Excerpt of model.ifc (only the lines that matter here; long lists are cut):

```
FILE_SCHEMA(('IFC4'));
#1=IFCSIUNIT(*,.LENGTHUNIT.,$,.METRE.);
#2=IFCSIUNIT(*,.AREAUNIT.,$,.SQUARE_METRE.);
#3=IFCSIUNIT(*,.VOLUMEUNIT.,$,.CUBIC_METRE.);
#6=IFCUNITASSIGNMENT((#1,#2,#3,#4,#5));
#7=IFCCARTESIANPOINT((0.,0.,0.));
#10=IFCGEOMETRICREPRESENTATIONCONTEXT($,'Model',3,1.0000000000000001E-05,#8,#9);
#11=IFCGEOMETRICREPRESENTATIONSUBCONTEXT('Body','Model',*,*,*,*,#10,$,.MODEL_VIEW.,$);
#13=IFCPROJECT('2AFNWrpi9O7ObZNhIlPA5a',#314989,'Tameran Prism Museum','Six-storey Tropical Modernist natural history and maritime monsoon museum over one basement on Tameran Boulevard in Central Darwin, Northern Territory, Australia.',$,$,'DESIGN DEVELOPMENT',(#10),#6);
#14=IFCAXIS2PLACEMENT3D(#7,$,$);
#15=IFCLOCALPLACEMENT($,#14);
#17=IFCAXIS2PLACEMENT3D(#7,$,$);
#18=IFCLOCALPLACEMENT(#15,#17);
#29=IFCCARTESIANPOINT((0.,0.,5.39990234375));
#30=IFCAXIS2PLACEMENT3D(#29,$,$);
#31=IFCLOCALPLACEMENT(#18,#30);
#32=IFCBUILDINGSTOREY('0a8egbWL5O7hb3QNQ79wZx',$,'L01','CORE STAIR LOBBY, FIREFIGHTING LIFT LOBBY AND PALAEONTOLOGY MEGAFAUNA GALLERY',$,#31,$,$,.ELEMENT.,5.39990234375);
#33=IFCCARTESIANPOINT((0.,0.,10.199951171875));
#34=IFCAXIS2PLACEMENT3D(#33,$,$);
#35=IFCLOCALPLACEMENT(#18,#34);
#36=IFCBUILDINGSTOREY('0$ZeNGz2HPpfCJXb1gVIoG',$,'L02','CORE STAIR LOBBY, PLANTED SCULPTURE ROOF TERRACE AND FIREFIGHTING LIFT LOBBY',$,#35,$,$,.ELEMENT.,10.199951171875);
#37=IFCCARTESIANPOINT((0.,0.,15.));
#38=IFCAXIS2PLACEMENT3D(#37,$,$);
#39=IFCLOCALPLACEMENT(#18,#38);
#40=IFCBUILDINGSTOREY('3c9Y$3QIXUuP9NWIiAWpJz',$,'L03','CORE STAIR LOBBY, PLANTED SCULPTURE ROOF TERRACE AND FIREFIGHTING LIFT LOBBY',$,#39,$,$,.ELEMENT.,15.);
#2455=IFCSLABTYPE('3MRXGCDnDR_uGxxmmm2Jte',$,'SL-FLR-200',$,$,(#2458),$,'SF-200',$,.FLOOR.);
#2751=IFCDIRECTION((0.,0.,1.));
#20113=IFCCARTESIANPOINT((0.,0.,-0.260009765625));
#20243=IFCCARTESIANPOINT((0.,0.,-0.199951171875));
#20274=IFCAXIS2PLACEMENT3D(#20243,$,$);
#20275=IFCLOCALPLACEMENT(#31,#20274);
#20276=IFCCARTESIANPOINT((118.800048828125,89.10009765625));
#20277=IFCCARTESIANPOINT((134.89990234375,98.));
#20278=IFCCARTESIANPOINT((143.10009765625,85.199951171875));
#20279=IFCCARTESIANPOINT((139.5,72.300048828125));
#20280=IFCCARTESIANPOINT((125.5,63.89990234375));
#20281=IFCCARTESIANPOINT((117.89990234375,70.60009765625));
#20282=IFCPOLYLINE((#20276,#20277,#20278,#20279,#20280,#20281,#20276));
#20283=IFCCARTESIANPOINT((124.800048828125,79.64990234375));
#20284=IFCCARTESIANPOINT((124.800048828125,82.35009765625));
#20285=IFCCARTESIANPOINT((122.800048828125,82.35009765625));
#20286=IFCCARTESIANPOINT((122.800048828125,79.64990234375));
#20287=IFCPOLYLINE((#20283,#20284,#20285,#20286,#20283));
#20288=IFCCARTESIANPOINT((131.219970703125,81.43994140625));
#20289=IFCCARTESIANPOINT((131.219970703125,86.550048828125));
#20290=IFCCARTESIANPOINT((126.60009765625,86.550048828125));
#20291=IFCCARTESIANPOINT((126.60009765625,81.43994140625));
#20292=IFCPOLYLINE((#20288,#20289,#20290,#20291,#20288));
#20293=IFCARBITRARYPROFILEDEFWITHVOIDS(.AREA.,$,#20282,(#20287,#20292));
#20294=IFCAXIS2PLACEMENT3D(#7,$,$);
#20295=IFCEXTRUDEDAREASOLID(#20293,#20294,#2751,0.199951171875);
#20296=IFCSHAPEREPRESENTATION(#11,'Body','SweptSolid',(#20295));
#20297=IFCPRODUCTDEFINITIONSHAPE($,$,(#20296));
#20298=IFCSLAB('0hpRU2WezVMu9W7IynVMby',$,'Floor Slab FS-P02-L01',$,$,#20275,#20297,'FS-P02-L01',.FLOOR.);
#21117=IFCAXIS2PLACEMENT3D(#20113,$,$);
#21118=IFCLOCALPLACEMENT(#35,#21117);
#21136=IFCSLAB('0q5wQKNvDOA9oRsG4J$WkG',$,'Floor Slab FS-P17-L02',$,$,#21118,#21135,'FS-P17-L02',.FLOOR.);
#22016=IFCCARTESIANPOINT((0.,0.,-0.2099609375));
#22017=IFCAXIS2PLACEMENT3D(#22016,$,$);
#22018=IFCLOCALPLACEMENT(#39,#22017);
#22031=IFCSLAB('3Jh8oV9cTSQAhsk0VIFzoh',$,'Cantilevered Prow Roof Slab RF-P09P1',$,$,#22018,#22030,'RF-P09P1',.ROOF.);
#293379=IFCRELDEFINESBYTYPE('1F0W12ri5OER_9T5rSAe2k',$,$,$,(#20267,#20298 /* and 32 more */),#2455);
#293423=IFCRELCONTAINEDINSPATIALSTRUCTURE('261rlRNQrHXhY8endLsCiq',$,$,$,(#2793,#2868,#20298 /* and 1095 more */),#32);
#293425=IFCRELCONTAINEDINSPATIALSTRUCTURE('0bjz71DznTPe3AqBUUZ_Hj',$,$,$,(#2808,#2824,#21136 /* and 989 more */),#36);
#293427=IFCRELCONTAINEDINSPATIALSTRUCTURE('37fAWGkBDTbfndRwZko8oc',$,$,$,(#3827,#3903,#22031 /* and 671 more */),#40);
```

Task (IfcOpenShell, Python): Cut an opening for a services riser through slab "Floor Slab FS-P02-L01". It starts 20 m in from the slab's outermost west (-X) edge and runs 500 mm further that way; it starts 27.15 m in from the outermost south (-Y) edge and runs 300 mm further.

```python
import numpy as np
import ifcopenshell
import ifcopenshell.api.feature
import ifcopenshell.api.geometry
import ifcopenshell.api.root
import ifcopenshell.geom
import ifcopenshell.util.placement
import ifcopenshell.util.representation
import ifcopenshell.util.shape
import ifcopenshell.util.unit

model = ifcopenshell.open("model.ifc")
unit_scale = ifcopenshell.util.unit.calculate_unit_scale(model)
settings = ifcopenshell.geom.settings()


def volume(element):
    """Net volume in cubic metres, openings subtracted."""
    shape = ifcopenshell.geom.create_shape(settings, element)
    return ifcopenshell.util.shape.get_volume(shape.geometry)


slab = model.by_guid("0hpRU2WezVMu9W7IynVMby")
before = volume(slab)

# Extent in the slab's own axes, in metres. The edges named are its -X and -Y sides.
slab_shape = ifcopenshell.geom.create_shape(settings, slab)
vertices = ifcopenshell.util.shape.get_vertices(slab_shape.geometry)
x_min, y_min, bottom = vertices.min(axis=0)
top = vertices[:, 2].max()

opening = ifcopenshell.api.root.create_entity(model, ifc_class="IfcOpeningElement", name="Services riser opening", predefined_type="OPENING")
context = ifcopenshell.util.representation.get_context(model, "Model", "Body", "MODEL_VIEW")
width, depth = 0.5, 0.3
outline = [(0.0, 0.0), (width, 0.0), (width, depth), (0.0, depth), (0.0, 0.0)]
# Overshoot both faces by 50 mm so the cut is clean.
shape = ifcopenshell.api.geometry.add_slab_representation(
    model, context=context, depth=top - bottom + 0.1, polyline=outline
)
ifcopenshell.api.geometry.assign_representation(model, product=opening, representation=shape)

matrix = ifcopenshell.util.placement.get_local_placement(slab.ObjectPlacement)
matrix[:, 3] = matrix @ np.append(np.array([x_min + 20, y_min + 27.15, bottom - 0.05]) / unit_scale, 1.0)
ifcopenshell.api.geometry.edit_object_placement(model, product=opening, matrix=matrix, is_si=False)
ifcopenshell.api.feature.add_feature(model, feature=opening, element=slab)

after = volume(slab)

print(f"slab volume {before:.3f} -> {after:.3f} m3")

model.write("model-out.ifc")
```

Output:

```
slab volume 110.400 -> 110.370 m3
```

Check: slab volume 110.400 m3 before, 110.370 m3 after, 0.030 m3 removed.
